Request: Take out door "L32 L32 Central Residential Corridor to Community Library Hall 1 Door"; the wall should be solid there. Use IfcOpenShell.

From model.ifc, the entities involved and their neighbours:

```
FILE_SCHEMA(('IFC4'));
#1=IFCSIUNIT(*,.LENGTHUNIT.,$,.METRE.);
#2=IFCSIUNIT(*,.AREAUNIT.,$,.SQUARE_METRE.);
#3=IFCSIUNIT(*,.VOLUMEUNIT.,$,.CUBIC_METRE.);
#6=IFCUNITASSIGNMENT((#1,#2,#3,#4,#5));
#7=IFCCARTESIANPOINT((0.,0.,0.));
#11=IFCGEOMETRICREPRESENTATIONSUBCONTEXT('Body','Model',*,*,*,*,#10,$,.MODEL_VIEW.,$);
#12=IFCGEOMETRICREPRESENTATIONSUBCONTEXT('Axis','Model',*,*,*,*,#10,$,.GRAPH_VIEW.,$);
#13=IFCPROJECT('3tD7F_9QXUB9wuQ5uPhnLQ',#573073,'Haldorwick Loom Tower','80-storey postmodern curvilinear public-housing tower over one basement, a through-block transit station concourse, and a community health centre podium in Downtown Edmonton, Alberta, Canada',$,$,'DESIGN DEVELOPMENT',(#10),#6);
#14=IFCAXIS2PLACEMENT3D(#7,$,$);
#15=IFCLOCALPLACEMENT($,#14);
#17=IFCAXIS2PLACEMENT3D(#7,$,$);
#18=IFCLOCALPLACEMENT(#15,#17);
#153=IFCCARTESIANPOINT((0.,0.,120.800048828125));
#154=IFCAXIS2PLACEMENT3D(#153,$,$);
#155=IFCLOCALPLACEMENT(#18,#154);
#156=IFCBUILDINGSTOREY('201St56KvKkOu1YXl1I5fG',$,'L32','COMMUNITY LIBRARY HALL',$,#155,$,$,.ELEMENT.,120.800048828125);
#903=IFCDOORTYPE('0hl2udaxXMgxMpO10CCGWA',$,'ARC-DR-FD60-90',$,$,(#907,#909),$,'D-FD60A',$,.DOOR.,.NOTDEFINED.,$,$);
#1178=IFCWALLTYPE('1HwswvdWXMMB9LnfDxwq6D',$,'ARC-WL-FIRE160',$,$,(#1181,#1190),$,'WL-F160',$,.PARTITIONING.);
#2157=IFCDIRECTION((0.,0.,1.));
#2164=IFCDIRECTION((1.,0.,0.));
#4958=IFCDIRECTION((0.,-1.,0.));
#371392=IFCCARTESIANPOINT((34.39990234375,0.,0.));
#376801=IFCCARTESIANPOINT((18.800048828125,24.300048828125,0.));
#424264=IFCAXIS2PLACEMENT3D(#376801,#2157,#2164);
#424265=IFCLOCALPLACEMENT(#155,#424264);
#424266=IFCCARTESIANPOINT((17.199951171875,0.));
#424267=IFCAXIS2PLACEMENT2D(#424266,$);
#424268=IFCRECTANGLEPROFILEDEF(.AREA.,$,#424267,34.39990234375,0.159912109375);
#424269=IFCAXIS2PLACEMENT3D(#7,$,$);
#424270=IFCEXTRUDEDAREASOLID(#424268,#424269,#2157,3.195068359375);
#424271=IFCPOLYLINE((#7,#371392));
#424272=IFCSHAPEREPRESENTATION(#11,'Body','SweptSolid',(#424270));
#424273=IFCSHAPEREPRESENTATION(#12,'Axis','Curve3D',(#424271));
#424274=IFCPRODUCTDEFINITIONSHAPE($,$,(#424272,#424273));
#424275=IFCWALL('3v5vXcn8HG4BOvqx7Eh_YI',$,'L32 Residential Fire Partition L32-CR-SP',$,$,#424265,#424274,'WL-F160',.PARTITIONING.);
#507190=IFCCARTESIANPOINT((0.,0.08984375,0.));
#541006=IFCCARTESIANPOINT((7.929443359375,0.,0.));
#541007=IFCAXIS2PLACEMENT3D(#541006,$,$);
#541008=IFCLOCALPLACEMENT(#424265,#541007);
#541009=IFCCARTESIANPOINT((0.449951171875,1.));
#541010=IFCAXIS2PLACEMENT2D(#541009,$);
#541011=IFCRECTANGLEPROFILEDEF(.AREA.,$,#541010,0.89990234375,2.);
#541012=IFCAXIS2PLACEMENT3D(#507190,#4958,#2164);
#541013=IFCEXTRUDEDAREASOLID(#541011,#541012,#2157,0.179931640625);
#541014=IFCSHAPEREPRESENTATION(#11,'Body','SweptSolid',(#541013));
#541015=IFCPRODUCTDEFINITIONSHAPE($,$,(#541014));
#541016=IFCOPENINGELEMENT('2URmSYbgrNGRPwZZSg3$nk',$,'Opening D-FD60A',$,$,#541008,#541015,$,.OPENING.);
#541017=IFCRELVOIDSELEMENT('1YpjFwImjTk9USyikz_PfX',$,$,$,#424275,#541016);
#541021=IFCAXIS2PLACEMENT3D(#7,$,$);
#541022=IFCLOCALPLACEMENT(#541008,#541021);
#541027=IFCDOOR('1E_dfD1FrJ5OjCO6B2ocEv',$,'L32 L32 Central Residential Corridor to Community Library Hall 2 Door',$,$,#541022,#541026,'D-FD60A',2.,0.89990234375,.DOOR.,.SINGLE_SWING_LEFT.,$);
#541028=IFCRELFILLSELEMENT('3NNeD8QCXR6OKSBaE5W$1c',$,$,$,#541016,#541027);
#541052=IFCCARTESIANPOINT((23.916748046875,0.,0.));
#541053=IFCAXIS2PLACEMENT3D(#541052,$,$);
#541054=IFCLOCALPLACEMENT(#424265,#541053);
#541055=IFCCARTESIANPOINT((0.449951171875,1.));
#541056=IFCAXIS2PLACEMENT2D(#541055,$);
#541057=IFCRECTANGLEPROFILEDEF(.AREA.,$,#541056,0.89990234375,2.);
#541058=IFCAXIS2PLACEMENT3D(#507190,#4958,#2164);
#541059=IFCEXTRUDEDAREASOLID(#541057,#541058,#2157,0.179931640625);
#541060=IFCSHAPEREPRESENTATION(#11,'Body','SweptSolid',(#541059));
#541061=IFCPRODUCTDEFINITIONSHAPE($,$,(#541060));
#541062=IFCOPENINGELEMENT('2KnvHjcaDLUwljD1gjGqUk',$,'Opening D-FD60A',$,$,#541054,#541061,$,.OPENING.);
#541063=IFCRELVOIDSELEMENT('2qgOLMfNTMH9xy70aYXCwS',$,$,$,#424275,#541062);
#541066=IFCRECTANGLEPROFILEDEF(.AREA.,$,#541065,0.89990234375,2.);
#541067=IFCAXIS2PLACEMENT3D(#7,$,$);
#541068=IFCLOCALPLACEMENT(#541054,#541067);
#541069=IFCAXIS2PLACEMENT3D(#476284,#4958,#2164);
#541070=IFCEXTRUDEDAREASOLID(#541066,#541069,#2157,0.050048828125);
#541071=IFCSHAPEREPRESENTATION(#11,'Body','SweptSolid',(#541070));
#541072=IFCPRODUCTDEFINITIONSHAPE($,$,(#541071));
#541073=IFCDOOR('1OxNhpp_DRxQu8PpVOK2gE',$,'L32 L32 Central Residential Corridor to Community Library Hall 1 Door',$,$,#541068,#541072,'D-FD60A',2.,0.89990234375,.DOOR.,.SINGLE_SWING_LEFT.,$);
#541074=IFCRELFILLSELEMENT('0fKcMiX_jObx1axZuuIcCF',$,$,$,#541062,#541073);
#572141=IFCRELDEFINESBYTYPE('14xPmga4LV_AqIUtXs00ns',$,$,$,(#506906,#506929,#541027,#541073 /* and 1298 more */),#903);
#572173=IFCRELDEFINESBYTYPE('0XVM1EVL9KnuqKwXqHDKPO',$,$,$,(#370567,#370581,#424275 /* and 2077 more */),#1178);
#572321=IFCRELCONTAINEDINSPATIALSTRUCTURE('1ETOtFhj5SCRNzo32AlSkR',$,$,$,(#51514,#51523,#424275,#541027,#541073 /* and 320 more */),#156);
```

```python
import ifcopenshell
import ifcopenshell.api.feature
import ifcopenshell.api.root
import ifcopenshell.geom
import ifcopenshell.util.shape

model = ifcopenshell.open("model.ifc")
settings = ifcopenshell.geom.settings()


def volume(element):
    """Net volume in cubic metres, openings subtracted."""
    shape = ifcopenshell.geom.create_shape(settings, element)
    return ifcopenshell.util.shape.get_volume(shape.geometry)


door = model.by_guid("1OxNhpp_DRxQu8PpVOK2gE")
opening = door.FillsVoids[0].RelatingOpeningElement
wall = opening.VoidsElements[0].RelatingBuildingElement
before = volume(wall)

ifcopenshell.api.root.remove_product(model, product=door)
ifcopenshell.api.feature.remove_feature(model, feature=opening)

after = volume(wall)

print(f"wall volume {before:.3f} -> {after:.3f} m3")

model.write("model_updated.ifc")
```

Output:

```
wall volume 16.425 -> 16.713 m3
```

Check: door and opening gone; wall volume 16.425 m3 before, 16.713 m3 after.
